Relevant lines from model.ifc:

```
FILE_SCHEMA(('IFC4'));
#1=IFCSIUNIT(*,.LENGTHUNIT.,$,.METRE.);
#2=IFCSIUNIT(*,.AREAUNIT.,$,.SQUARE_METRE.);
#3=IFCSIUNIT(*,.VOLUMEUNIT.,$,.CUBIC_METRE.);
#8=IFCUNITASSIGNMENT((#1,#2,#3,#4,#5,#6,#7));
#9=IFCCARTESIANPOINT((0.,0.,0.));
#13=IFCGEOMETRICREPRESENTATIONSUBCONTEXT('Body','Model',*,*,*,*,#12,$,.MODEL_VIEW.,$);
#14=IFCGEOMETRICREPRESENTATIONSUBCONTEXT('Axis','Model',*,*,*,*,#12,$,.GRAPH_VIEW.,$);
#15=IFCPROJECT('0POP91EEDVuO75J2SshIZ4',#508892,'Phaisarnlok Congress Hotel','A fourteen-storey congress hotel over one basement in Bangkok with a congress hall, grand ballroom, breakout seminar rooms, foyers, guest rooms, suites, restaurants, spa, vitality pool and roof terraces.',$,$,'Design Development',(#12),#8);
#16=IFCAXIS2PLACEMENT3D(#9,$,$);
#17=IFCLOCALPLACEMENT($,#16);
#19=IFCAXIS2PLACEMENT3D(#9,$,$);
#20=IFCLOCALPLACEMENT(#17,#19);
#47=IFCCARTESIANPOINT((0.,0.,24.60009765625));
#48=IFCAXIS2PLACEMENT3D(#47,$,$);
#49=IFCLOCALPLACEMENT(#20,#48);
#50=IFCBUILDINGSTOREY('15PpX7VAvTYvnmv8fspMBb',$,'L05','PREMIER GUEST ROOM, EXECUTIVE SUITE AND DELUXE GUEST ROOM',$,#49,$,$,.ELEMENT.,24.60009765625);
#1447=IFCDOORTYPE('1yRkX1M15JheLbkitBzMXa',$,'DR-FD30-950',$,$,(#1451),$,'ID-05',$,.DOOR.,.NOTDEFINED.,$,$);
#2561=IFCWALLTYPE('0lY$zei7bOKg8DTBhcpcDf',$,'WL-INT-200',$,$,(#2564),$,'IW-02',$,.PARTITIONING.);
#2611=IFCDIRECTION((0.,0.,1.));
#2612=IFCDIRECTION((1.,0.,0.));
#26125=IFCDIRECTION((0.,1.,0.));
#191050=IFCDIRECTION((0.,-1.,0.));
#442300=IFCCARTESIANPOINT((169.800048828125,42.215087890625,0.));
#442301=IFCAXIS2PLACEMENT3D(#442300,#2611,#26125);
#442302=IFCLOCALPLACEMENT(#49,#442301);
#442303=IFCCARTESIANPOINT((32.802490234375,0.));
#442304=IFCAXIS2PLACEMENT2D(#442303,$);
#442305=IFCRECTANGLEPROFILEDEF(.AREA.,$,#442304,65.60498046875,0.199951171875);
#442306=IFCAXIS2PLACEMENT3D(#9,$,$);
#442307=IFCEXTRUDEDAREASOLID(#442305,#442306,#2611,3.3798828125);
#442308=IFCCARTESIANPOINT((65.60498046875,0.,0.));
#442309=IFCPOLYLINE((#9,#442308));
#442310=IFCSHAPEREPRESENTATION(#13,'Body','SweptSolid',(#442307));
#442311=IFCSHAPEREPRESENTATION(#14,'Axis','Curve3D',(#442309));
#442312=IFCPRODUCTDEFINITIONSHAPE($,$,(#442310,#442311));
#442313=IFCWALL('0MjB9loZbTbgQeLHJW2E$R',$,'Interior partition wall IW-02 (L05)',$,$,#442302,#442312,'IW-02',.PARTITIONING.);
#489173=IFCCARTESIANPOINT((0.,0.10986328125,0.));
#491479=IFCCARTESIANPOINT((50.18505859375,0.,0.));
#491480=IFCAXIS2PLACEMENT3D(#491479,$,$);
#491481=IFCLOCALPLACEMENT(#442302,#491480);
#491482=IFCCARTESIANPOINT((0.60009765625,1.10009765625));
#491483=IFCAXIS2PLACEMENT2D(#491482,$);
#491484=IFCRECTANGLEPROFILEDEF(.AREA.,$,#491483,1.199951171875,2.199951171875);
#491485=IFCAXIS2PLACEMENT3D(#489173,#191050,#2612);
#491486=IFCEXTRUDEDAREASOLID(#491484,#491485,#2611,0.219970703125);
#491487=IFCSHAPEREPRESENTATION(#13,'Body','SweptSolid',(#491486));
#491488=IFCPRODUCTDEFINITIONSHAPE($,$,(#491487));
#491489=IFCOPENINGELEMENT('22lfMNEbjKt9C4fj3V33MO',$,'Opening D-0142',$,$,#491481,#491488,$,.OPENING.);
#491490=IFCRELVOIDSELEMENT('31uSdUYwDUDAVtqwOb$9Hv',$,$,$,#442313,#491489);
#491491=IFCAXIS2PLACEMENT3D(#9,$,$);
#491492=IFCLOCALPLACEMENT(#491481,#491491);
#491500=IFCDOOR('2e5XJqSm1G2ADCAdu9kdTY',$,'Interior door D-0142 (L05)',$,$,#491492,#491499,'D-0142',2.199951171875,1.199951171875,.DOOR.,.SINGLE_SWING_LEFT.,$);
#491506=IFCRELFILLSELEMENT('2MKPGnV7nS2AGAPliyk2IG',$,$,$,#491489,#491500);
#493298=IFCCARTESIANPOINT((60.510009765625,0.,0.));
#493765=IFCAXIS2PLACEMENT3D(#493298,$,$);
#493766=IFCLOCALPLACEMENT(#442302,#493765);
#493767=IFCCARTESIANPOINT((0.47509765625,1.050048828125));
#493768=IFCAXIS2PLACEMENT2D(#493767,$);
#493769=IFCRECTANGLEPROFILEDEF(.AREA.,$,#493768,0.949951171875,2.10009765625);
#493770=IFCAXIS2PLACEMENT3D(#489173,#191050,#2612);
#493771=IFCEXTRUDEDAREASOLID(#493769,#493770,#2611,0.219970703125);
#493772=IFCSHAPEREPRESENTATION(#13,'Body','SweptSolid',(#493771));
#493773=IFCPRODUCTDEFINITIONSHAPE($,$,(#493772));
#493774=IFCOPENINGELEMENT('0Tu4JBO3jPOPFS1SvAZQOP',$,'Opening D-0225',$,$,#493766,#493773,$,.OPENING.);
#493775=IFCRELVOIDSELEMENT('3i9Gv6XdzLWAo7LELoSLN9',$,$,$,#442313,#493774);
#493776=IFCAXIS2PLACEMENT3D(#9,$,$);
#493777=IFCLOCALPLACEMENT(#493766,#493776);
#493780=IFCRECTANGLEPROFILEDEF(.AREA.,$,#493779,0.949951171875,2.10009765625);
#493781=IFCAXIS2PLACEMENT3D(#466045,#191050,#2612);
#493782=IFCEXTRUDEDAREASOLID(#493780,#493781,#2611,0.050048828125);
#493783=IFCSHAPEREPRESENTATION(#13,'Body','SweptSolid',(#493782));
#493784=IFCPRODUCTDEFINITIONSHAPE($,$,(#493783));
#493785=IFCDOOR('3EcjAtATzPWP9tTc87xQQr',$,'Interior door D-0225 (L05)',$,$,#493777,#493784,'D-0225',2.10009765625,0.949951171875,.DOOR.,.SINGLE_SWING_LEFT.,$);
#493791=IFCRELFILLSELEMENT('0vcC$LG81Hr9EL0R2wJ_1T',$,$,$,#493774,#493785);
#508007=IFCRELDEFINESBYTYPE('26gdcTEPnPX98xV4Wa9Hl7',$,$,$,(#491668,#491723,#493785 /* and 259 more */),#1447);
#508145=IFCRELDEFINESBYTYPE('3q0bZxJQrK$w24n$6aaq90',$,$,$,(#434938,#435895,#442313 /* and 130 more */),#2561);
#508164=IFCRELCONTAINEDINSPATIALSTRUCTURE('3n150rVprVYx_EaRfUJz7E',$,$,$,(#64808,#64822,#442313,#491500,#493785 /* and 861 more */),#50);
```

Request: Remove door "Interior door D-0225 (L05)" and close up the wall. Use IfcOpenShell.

```python
import ifcopenshell
import ifcopenshell.api.feature
import ifcopenshell.api.root
import ifcopenshell.geom
import ifcopenshell.util.shape

model = ifcopenshell.open("model.ifc")
settings = ifcopenshell.geom.settings()


def volume(element):
    """Net volume in cubic metres, openings subtracted."""
    shape = ifcopenshell.geom.create_shape(settings, element)
    return ifcopenshell.util.shape.get_volume(shape.geometry)


door = model.by_id(493785)
opening = door.FillsVoids[0].RelatingOpeningElement
wall = opening.VoidsElements[0].RelatingBuildingElement
before = volume(wall)

ifcopenshell.api.root.remove_product(model, product=door)
ifcopenshell.api.feature.remove_feature(model, feature=opening)

after = volume(wall)

print(f"wall volume {before:.3f} -> {after:.3f} m3")

model.write("model_v2.ifc")
```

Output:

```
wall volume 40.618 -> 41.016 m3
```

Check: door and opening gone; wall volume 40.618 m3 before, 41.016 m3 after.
